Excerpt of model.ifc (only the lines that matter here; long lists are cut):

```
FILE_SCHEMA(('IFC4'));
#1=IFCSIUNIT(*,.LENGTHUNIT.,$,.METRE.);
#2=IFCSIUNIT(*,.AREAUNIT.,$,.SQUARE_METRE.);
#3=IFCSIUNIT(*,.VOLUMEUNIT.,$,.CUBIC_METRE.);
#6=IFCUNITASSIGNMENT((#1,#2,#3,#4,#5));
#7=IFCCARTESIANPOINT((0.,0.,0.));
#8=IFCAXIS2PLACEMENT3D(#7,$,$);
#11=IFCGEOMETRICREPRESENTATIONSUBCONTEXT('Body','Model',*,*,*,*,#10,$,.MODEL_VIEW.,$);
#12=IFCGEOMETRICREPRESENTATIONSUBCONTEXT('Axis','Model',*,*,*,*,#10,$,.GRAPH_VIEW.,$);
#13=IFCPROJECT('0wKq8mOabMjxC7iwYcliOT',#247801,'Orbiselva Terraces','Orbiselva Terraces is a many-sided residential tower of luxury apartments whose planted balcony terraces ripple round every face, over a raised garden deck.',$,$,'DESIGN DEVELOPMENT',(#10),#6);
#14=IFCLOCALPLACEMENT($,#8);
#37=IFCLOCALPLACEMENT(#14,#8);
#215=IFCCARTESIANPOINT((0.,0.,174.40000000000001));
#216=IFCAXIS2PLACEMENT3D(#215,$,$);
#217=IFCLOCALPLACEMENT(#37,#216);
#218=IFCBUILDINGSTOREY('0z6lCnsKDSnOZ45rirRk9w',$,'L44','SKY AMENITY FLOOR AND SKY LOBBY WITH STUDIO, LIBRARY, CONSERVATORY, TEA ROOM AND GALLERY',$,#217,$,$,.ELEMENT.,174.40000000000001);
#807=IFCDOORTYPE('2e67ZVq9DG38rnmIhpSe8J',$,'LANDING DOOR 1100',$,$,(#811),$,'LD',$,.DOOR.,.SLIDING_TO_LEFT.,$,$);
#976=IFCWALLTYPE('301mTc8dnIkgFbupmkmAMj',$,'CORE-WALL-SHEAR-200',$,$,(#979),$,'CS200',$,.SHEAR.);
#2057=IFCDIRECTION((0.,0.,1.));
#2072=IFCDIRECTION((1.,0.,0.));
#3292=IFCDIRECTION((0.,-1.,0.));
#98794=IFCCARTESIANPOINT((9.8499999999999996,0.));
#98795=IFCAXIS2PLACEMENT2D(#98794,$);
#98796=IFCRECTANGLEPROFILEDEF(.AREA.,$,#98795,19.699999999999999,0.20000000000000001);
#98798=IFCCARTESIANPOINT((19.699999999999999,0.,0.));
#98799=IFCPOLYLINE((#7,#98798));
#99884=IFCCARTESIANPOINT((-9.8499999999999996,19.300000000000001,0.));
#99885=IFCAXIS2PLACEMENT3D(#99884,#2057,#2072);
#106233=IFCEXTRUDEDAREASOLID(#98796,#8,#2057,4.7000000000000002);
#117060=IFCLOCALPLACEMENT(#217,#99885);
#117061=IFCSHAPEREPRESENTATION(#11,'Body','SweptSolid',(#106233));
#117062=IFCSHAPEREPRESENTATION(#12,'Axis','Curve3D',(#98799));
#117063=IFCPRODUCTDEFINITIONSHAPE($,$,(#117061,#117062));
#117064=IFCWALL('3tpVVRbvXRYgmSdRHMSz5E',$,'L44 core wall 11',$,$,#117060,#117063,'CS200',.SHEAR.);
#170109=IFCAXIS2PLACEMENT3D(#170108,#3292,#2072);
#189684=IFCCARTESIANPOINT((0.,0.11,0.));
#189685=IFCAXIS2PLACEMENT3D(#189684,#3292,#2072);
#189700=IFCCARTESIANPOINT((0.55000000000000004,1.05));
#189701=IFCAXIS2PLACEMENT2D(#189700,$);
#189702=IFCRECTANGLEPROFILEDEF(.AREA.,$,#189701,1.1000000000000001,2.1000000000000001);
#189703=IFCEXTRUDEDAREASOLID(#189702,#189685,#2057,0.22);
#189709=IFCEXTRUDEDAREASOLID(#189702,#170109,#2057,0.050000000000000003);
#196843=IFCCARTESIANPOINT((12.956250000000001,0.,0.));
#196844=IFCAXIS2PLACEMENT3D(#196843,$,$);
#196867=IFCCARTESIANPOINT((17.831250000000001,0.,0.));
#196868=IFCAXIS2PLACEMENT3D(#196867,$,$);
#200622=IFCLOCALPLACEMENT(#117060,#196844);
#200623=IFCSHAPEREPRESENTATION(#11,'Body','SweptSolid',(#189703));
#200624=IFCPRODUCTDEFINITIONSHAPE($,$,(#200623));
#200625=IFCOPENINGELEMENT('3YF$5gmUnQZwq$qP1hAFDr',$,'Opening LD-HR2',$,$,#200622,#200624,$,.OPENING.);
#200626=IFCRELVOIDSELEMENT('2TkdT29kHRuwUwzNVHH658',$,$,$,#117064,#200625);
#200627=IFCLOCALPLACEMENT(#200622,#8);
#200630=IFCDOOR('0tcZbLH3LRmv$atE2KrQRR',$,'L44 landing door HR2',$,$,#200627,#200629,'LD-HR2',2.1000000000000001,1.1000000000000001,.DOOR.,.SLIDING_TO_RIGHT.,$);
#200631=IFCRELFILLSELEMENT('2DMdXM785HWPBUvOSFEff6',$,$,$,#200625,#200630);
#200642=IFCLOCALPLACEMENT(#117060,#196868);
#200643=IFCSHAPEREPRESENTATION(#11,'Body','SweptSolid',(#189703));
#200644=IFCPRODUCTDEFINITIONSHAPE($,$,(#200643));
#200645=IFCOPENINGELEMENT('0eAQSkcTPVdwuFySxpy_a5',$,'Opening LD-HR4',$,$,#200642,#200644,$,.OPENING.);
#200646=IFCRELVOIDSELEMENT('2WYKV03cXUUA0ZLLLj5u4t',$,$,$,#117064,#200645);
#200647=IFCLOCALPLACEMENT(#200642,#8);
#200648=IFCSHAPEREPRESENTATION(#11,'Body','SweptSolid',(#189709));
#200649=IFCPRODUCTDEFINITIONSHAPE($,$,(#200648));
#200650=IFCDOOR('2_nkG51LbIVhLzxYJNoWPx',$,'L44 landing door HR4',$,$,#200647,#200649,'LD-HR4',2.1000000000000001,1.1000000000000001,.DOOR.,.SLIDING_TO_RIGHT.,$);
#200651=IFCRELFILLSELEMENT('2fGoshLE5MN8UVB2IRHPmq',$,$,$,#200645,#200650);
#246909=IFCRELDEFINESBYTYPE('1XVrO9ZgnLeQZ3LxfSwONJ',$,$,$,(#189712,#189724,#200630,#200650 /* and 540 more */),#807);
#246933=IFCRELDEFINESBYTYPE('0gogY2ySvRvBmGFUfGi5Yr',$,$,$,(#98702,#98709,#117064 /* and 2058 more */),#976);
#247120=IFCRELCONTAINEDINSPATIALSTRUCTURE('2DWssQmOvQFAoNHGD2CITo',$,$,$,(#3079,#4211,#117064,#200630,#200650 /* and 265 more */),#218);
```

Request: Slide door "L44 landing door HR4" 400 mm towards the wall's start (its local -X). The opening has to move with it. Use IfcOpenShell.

```python
import ifcopenshell
import ifcopenshell.api.geometry
import ifcopenshell.util.placement
import ifcopenshell.util.unit

model = ifcopenshell.open("model.ifc")
unit_scale = ifcopenshell.util.unit.calculate_unit_scale(model)

door = model.by_guid("2_nkG51LbIVhLzxYJNoWPx")
opening = door.FillsVoids[0].RelatingOpeningElement
wall = opening.VoidsElements[0].RelatingBuildingElement

wall_matrix = ifcopenshell.util.placement.get_local_placement(wall.ObjectPlacement)
shift = wall_matrix[:3, 0] * -0.4 / unit_scale
before = ifcopenshell.util.placement.get_local_placement(door.ObjectPlacement)[:3, 3].copy()

# The door is placed relative to its opening, so it follows when the opening moves.
matrix = ifcopenshell.util.placement.get_local_placement(opening.ObjectPlacement)
matrix[:3, 3] += shift
ifcopenshell.api.geometry.edit_object_placement(
    model, product=opening, matrix=matrix, is_si=False, should_transform_children=True
)

after = ifcopenshell.util.placement.get_local_placement(door.ObjectPlacement)[:3, 3]
print("door moved by", (after - before).round(3) + 0.0)

model.write("model_updated.ifc")
```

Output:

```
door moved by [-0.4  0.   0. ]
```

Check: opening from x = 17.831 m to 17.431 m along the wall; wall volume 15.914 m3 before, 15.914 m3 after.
